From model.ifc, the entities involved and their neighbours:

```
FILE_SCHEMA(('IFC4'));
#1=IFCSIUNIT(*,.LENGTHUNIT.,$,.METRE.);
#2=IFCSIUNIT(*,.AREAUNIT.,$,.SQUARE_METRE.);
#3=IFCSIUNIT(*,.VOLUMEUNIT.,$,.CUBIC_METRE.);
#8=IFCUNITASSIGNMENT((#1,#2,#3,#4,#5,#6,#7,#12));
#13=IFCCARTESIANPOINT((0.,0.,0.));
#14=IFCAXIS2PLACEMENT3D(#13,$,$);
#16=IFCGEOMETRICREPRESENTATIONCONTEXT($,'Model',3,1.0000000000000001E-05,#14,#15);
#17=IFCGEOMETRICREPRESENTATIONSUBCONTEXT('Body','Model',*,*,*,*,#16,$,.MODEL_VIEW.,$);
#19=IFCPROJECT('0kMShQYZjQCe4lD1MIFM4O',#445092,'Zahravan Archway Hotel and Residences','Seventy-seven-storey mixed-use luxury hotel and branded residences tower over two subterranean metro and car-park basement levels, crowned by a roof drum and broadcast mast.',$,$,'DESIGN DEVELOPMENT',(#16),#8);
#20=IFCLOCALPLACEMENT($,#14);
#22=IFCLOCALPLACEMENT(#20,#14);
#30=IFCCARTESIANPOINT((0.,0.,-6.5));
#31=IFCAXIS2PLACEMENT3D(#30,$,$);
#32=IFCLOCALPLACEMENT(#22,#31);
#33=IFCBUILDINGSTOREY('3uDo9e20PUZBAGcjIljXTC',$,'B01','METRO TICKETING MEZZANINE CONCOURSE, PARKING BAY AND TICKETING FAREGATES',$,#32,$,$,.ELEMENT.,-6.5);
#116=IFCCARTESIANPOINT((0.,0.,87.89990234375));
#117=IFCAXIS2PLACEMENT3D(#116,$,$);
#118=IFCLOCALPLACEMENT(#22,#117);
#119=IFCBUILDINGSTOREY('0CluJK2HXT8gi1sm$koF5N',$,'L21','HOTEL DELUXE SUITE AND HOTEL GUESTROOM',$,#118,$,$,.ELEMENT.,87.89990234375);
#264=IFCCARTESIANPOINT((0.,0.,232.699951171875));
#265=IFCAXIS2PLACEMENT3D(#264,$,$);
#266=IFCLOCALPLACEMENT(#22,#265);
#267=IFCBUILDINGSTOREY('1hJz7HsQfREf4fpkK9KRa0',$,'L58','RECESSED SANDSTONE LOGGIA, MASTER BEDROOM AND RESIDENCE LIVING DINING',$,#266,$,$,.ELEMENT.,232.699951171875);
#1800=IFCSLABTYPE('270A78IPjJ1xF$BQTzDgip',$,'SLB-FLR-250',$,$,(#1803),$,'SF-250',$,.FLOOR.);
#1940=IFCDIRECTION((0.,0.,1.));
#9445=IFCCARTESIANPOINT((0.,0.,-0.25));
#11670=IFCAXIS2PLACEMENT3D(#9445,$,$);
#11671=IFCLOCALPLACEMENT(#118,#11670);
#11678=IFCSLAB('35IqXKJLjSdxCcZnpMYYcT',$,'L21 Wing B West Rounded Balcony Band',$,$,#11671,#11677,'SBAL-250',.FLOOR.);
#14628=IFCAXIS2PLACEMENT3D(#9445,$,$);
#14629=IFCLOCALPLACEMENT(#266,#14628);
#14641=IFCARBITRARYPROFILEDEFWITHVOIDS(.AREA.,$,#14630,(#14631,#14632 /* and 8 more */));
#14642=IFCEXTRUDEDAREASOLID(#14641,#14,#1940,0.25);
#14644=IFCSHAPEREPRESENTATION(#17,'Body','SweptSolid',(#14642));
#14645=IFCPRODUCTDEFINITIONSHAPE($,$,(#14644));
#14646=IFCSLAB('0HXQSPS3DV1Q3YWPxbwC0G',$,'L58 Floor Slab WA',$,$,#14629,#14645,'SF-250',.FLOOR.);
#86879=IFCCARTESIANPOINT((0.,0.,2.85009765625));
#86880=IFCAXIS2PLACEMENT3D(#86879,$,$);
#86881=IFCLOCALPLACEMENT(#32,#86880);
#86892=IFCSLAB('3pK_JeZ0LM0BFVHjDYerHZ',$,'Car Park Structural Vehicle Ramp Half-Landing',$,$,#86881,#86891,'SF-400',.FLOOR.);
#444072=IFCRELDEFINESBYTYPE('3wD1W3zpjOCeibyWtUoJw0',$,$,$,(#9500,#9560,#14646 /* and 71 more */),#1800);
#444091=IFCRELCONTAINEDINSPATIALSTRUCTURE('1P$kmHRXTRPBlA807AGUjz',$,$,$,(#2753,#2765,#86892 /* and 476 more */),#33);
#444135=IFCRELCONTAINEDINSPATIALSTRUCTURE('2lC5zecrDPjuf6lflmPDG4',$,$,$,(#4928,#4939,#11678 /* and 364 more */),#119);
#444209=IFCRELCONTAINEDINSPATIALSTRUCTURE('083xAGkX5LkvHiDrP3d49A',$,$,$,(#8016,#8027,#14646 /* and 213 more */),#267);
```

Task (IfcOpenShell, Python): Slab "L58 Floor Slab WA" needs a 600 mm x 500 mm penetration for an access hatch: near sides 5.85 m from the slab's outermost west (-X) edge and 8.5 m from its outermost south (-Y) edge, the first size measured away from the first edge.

```python
import numpy as np
import ifcopenshell
import ifcopenshell.api.feature
import ifcopenshell.api.geometry
import ifcopenshell.api.root
import ifcopenshell.geom
import ifcopenshell.util.placement
import ifcopenshell.util.representation
import ifcopenshell.util.shape
import ifcopenshell.util.unit

model = ifcopenshell.open("model.ifc")
unit_scale = ifcopenshell.util.unit.calculate_unit_scale(model)
settings = ifcopenshell.geom.settings()


def volume(element):
    """Net volume in cubic metres, openings subtracted."""
    shape = ifcopenshell.geom.create_shape(settings, element)
    return ifcopenshell.util.shape.get_volume(shape.geometry)


slab = model.by_guid("0HXQSPS3DV1Q3YWPxbwC0G")
before = volume(slab)

# Extent in the slab's own axes, in metres. The edges named are its -X and -Y sides.
slab_shape = ifcopenshell.geom.create_shape(settings, slab)
vertices = ifcopenshell.util.shape.get_vertices(slab_shape.geometry)
x_min, y_min, bottom = vertices.min(axis=0)
top = vertices[:, 2].max()

opening = ifcopenshell.api.root.create_entity(model, ifc_class="IfcOpeningElement", name="Access hatch opening", predefined_type="OPENING")
context = ifcopenshell.util.representation.get_context(model, "Model", "Body", "MODEL_VIEW")
width, depth = 0.6, 0.5
outline = [(0.0, 0.0), (width, 0.0), (width, depth), (0.0, depth), (0.0, 0.0)]
# Overshoot both faces by 50 mm so the cut is clean.
shape = ifcopenshell.api.geometry.add_slab_representation(
    model, context=context, depth=top - bottom + 0.1, polyline=outline
)
ifcopenshell.api.geometry.assign_representation(model, product=opening, representation=shape)

matrix = ifcopenshell.util.placement.get_local_placement(slab.ObjectPlacement)
matrix[:, 3] = matrix @ np.append(np.array([x_min + 5.85, y_min + 8.5, bottom - 0.05]) / unit_scale, 1.0)
ifcopenshell.api.geometry.edit_object_placement(model, product=opening, matrix=matrix, is_si=False)
ifcopenshell.api.feature.add_feature(model, feature=opening, element=slab)

after = volume(slab)

print(f"slab volume {before:.3f} -> {after:.3f} m3")

model.write("model_edited.ifc")
```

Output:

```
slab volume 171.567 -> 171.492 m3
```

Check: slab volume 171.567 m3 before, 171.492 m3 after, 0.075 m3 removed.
